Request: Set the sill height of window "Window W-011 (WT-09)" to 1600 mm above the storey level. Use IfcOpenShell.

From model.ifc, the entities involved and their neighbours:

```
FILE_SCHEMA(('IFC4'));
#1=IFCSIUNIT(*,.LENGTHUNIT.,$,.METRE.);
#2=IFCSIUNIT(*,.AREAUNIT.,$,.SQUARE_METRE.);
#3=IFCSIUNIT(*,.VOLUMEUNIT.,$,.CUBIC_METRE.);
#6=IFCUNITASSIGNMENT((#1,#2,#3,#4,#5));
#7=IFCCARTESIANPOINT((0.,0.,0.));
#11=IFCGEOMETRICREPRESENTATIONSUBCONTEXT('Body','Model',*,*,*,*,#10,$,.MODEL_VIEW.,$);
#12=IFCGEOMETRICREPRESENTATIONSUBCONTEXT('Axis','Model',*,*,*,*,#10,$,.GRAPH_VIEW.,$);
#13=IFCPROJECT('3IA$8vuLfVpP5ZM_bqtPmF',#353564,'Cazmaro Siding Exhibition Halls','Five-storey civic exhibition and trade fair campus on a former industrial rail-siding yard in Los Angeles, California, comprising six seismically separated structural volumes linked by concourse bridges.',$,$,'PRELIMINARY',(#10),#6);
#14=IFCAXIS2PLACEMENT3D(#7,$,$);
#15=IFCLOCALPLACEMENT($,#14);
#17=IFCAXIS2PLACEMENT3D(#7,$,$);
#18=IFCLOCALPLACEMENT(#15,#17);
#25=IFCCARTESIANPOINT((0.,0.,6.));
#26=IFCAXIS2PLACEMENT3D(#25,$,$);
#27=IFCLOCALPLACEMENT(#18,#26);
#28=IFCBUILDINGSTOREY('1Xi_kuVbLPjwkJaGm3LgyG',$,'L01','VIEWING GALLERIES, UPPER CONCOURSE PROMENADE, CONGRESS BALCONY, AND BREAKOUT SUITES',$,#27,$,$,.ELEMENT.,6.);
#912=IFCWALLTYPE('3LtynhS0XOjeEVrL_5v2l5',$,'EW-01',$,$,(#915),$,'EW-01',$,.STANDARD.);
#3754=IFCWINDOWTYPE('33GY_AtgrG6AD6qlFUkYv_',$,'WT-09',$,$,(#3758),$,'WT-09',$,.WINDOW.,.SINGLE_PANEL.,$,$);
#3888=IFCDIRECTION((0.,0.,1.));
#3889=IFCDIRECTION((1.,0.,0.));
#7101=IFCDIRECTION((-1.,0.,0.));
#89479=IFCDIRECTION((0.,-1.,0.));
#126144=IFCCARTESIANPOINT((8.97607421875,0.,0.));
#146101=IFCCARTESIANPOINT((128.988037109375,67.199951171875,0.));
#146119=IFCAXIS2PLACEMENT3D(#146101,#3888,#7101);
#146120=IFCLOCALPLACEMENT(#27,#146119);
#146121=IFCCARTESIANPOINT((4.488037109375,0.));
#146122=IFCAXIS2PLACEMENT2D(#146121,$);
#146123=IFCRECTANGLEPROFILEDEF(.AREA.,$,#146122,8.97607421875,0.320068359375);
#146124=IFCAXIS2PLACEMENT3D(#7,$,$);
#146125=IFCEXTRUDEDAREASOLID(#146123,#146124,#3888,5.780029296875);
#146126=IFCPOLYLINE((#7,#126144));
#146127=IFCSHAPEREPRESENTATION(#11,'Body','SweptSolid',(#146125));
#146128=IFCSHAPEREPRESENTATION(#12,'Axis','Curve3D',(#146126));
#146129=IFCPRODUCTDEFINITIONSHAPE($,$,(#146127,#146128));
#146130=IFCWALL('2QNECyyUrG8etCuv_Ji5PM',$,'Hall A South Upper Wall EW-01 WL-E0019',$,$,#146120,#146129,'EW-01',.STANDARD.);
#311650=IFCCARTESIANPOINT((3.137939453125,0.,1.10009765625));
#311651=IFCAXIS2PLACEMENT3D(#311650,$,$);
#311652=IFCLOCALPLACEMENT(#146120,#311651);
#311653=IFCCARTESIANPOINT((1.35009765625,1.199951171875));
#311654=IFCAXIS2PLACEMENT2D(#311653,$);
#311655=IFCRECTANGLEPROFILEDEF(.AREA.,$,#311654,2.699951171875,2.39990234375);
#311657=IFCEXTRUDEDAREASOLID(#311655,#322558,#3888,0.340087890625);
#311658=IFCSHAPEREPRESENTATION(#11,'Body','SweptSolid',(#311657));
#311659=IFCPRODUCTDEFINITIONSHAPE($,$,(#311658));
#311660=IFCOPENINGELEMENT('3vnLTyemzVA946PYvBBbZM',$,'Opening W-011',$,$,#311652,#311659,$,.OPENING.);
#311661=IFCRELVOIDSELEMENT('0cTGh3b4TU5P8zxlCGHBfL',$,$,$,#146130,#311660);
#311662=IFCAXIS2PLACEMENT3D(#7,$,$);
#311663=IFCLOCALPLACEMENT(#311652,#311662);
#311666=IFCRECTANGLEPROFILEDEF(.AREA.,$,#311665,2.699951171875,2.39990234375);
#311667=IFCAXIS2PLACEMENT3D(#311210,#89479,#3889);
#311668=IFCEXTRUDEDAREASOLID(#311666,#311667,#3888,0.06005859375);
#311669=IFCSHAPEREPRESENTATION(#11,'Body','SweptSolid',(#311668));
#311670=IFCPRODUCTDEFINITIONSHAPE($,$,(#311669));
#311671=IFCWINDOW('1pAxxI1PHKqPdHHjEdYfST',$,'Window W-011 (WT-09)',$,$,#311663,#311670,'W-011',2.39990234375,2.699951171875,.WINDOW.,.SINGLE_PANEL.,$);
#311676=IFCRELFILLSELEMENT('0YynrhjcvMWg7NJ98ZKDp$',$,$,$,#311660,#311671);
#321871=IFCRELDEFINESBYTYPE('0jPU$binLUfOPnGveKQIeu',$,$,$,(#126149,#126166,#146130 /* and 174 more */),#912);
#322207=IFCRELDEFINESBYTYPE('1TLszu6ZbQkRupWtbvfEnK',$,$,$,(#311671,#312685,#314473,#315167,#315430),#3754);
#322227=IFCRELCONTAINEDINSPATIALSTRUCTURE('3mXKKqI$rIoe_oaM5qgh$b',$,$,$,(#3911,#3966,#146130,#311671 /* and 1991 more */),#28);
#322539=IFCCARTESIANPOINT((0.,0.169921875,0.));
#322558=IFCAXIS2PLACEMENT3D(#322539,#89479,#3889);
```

```python
import numpy as np
import ifcopenshell
import ifcopenshell.api.geometry
import ifcopenshell.geom
import ifcopenshell.util.element
import ifcopenshell.util.placement
import ifcopenshell.util.shape
import ifcopenshell.util.unit

model = ifcopenshell.open("model.ifc")
unit_scale = ifcopenshell.util.unit.calculate_unit_scale(model)

window = model.by_guid("1pAxxI1PHKqPdHHjEdYfST")
opening = window.FillsVoids[0].RelatingOpeningElement
storey = ifcopenshell.util.element.get_container(window, ifc_class="IfcBuildingStorey")
level = ifcopenshell.util.placement.get_local_placement(storey.ObjectPlacement)[2, 3]

# The opening's origin need not be at the sill, so measure its lowest point.
shape = ifcopenshell.geom.create_shape(ifcopenshell.geom.settings(), opening)
bottom = ifcopenshell.util.shape.get_shape_bottom_elevation(shape, shape.geometry) / unit_scale
dz = level + 1.6 - bottom

shift = np.array([0.0, 0.0, dz])
# The window is placed relative to its opening, so it follows when the opening moves.
matrix = ifcopenshell.util.placement.get_local_placement(opening.ObjectPlacement)
matrix[:3, 3] += shift
ifcopenshell.api.geometry.edit_object_placement(
    model, product=opening, matrix=matrix, is_si=False, should_transform_children=True
)

print(f"moved by {dz * unit_scale:+.3f} m")

model.write("model_edited.ifc")
```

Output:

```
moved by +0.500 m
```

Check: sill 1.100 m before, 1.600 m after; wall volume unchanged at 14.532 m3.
